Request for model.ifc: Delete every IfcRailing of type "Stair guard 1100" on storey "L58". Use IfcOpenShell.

First a look at what the model holds.

```python
import ifcopenshell
import ifcopenshell.util.element

model = ifcopenshell.open("model.ifc")
print(model.schema)
storey = next(s for s in model.by_type("IfcBuildingStorey") if s.Name == "L58")
railings = [e for e in ifcopenshell.util.element.get_decomposition(storey) if e.is_a("IfcRailing")]
seen = {}
for e in railings:
    element_type = ifcopenshell.util.element.get_type(e)
    name = element_type.Name if element_type not in (None, e) else None
    seen[name] = seen.get(name, 0) + 1
for name, count in sorted(seen.items(), key=str):
    print(count, "x", name)
```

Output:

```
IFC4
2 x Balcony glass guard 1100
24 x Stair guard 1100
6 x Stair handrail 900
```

```python
import ifcopenshell
import ifcopenshell.api.root
import ifcopenshell.util.element

model = ifcopenshell.open("model.ifc")

storey = next(s for s in model.by_type("IfcBuildingStorey") if s.Name == "L58")
railings = [e for e in ifcopenshell.util.element.get_decomposition(storey) if e.is_a("IfcRailing")]
targets = [e for e in railings if (t := ifcopenshell.util.element.get_type(e)) not in (None, e) and t.Name == "Stair guard 1100"]

for e in targets:
    ifcopenshell.api.root.remove_product(model, product=e)
print(len(targets), "removed")

model.write("model_v2.ifc")
```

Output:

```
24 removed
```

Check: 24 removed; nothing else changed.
